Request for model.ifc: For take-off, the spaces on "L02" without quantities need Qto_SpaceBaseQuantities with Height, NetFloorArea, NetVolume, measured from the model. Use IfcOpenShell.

First a look at what the model holds.

```python
import ifcopenshell
import ifcopenshell.util.element
import ifcopenshell.util.unit

model = ifcopenshell.open("model.ifc")
print(model.schema)
for unit_type in ("LENGTHUNIT", "AREAUNIT", "VOLUMEUNIT"):
    print(unit_type, ifcopenshell.util.unit.calculate_unit_scale(model, unit_type))
storey = next(s for s in model.by_type("IfcBuildingStorey") if s.Name == "L02")
spaces = [e for e in ifcopenshell.util.element.get_decomposition(storey) if e.is_a("IfcSpace")]
for e in sorted(spaces, key=lambda e: e.id()):
    print(e.id(), e.is_a(), e.Name, list(ifcopenshell.util.element.get_psets(e, qtos_only=True)), sep=" | ")
```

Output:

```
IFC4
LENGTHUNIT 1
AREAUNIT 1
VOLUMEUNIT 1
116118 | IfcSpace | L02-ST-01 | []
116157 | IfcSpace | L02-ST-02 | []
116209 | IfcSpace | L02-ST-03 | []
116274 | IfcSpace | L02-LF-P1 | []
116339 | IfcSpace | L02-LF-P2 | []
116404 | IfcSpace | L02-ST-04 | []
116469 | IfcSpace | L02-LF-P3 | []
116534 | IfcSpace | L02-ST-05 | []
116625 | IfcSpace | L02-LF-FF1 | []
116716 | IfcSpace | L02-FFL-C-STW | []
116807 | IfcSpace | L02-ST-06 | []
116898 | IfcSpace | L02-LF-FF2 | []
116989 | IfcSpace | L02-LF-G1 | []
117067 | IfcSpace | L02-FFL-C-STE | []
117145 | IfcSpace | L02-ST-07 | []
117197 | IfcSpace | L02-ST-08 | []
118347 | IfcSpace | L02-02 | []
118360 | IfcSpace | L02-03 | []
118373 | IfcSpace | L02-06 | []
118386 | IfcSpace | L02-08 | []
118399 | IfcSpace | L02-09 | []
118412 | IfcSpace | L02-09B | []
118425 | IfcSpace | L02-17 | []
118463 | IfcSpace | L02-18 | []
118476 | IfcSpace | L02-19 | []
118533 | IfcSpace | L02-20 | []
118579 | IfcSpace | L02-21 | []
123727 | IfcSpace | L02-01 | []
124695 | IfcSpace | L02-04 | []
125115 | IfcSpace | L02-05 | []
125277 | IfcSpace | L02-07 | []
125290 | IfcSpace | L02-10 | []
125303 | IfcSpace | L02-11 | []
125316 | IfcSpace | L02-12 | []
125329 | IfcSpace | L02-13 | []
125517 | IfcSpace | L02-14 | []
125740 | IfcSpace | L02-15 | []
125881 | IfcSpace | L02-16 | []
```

```python
import ifcopenshell
import ifcopenshell.api.pset
import ifcopenshell.geom
import ifcopenshell.util.element
import ifcopenshell.util.shape
import ifcopenshell.util.unit

model = ifcopenshell.open("model.ifc")
unit_scale = ifcopenshell.util.unit.calculate_unit_scale(model)
area_scale = ifcopenshell.util.unit.calculate_unit_scale(model, "AREAUNIT")
volume_scale = ifcopenshell.util.unit.calculate_unit_scale(model, "VOLUMEUNIT")
settings = ifcopenshell.geom.settings()

storey = next(s for s in model.by_type("IfcBuildingStorey") if s.Name == "L02")
spaces = [e for e in ifcopenshell.util.element.get_decomposition(storey) if e.is_a("IfcSpace")]

for e in sorted(spaces, key=lambda e: e.id()):
    if ifcopenshell.util.element.get_psets(e, qtos_only=True, should_inherit=False):
        continue
    # Geometry comes back in metres, in the element's own axes.
    shape = ifcopenshell.geom.create_shape(settings, e)
    values = {
        "Height": ifcopenshell.util.shape.get_z(shape.geometry) / unit_scale,
        "NetFloorArea": ifcopenshell.util.shape.get_footprint_area(shape.geometry) / area_scale,
        "NetVolume": ifcopenshell.util.shape.get_volume(shape.geometry) / volume_scale,
    }
    qto = ifcopenshell.api.pset.add_qto(model, product=e, name="Qto_SpaceBaseQuantities")
    ifcopenshell.api.pset.edit_qto(model, qto=qto, properties=values)
    print(e.id(), {k: round(v, 3) for k, v in values.items()})

model.write("model-out.ifc")
```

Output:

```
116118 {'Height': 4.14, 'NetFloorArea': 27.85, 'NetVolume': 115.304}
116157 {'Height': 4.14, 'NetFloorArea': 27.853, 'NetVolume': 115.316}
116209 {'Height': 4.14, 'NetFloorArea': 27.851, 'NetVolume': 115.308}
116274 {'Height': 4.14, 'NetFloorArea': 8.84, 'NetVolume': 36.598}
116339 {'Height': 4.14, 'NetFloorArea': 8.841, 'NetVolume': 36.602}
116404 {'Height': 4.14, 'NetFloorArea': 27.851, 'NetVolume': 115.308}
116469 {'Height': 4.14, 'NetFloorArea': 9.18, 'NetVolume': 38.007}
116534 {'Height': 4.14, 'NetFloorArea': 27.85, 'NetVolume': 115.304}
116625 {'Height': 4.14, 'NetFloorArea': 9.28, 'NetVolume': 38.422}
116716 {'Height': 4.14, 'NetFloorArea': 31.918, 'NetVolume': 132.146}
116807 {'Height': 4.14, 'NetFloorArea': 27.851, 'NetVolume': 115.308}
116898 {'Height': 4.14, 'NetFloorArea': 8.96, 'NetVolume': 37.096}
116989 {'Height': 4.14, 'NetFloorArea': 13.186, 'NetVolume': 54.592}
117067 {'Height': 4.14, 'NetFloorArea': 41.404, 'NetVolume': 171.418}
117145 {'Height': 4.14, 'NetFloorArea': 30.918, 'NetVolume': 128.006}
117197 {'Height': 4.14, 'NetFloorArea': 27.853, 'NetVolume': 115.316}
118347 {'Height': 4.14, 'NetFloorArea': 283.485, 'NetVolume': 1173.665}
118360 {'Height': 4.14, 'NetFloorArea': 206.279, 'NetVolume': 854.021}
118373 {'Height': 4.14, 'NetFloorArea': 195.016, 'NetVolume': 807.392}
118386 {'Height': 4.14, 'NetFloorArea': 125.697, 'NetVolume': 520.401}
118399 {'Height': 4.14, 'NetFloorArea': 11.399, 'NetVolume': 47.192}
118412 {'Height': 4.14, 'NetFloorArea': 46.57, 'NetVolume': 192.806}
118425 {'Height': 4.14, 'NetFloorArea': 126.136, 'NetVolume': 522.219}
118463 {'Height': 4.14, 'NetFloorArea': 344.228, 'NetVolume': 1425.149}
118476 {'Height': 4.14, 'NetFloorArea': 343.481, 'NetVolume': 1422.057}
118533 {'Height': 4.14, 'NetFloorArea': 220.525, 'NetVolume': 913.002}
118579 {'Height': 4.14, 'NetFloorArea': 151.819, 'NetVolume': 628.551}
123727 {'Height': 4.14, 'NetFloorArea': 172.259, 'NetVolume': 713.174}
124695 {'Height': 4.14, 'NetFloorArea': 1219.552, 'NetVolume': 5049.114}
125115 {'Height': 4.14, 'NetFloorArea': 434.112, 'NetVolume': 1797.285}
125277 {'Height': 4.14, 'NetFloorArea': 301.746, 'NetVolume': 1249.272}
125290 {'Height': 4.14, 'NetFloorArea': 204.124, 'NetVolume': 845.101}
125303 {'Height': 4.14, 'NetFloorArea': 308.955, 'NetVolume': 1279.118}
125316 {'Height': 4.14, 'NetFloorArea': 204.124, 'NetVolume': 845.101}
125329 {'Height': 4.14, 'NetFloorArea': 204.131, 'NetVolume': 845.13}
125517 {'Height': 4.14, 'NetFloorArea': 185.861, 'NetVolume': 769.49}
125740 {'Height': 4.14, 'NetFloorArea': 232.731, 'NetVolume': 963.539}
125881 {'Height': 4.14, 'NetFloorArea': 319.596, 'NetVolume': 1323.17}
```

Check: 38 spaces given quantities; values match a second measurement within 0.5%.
